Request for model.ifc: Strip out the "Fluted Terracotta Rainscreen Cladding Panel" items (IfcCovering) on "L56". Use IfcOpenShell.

First a look at what the model holds.

```python
import ifcopenshell
import ifcopenshell.util.element

model = ifcopenshell.open("model.ifc")
print(model.schema)
storey = next(s for s in model.by_type("IfcBuildingStorey") if s.Name == "L56")
coverings = [e for e in ifcopenshell.util.element.get_decomposition(storey) if e.is_a("IfcCovering")]
seen = {}
for e in coverings:
    element_type = ifcopenshell.util.element.get_type(e)
    name = element_type.Name if element_type not in (None, e) else None
    seen[name] = seen.get(name, 0) + 1
for name, count in sorted(seen.items(), key=str):
    print(count, "x", name)
```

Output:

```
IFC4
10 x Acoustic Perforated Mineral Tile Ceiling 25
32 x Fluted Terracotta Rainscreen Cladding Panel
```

```python
import ifcopenshell
import ifcopenshell.api.root
import ifcopenshell.util.element

model = ifcopenshell.open("model.ifc")

storey = next(s for s in model.by_type("IfcBuildingStorey") if s.Name == "L56")
coverings = [e for e in ifcopenshell.util.element.get_decomposition(storey) if e.is_a("IfcCovering")]
targets = [e for e in coverings if (t := ifcopenshell.util.element.get_type(e)) not in (None, e) and t.Name == "Fluted Terracotta Rainscreen Cladding Panel"]

for e in targets:
    ifcopenshell.api.root.remove_product(model, product=e)
print(len(targets), "removed")

model.write("model-out.ifc")
```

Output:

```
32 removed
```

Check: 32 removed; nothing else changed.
